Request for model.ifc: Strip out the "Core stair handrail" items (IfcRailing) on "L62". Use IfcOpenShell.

First a look at what the model holds.

```python
import ifcopenshell
import ifcopenshell.util.element

model = ifcopenshell.open("model.ifc")
print(model.schema)
storey = next(s for s in model.by_type("IfcBuildingStorey") if s.Name == "L62")
railings = [e for e in ifcopenshell.util.element.get_decomposition(storey) if e.is_a("IfcRailing")]
seen = {}
for e in railings:
    element_type = ifcopenshell.util.element.get_type(e)
    name = element_type.Name if element_type not in (None, e) else None
    seen[name] = seen.get(name, 0) + 1
for name, count in sorted(seen.items(), key=str):
    print(count, "x", name)
```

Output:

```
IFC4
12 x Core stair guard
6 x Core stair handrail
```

```python
import ifcopenshell
import ifcopenshell.api.root
import ifcopenshell.util.element

model = ifcopenshell.open("model.ifc")

storey = next(s for s in model.by_type("IfcBuildingStorey") if s.Name == "L62")
railings = [e for e in ifcopenshell.util.element.get_decomposition(storey) if e.is_a("IfcRailing")]
targets = [e for e in railings if (t := ifcopenshell.util.element.get_type(e)) not in (None, e) and t.Name == "Core stair handrail"]

for e in targets:
    ifcopenshell.api.root.remove_product(model, product=e)
print(len(targets), "removed")

model.write("model_edited.ifc")
```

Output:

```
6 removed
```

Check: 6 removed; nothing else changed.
